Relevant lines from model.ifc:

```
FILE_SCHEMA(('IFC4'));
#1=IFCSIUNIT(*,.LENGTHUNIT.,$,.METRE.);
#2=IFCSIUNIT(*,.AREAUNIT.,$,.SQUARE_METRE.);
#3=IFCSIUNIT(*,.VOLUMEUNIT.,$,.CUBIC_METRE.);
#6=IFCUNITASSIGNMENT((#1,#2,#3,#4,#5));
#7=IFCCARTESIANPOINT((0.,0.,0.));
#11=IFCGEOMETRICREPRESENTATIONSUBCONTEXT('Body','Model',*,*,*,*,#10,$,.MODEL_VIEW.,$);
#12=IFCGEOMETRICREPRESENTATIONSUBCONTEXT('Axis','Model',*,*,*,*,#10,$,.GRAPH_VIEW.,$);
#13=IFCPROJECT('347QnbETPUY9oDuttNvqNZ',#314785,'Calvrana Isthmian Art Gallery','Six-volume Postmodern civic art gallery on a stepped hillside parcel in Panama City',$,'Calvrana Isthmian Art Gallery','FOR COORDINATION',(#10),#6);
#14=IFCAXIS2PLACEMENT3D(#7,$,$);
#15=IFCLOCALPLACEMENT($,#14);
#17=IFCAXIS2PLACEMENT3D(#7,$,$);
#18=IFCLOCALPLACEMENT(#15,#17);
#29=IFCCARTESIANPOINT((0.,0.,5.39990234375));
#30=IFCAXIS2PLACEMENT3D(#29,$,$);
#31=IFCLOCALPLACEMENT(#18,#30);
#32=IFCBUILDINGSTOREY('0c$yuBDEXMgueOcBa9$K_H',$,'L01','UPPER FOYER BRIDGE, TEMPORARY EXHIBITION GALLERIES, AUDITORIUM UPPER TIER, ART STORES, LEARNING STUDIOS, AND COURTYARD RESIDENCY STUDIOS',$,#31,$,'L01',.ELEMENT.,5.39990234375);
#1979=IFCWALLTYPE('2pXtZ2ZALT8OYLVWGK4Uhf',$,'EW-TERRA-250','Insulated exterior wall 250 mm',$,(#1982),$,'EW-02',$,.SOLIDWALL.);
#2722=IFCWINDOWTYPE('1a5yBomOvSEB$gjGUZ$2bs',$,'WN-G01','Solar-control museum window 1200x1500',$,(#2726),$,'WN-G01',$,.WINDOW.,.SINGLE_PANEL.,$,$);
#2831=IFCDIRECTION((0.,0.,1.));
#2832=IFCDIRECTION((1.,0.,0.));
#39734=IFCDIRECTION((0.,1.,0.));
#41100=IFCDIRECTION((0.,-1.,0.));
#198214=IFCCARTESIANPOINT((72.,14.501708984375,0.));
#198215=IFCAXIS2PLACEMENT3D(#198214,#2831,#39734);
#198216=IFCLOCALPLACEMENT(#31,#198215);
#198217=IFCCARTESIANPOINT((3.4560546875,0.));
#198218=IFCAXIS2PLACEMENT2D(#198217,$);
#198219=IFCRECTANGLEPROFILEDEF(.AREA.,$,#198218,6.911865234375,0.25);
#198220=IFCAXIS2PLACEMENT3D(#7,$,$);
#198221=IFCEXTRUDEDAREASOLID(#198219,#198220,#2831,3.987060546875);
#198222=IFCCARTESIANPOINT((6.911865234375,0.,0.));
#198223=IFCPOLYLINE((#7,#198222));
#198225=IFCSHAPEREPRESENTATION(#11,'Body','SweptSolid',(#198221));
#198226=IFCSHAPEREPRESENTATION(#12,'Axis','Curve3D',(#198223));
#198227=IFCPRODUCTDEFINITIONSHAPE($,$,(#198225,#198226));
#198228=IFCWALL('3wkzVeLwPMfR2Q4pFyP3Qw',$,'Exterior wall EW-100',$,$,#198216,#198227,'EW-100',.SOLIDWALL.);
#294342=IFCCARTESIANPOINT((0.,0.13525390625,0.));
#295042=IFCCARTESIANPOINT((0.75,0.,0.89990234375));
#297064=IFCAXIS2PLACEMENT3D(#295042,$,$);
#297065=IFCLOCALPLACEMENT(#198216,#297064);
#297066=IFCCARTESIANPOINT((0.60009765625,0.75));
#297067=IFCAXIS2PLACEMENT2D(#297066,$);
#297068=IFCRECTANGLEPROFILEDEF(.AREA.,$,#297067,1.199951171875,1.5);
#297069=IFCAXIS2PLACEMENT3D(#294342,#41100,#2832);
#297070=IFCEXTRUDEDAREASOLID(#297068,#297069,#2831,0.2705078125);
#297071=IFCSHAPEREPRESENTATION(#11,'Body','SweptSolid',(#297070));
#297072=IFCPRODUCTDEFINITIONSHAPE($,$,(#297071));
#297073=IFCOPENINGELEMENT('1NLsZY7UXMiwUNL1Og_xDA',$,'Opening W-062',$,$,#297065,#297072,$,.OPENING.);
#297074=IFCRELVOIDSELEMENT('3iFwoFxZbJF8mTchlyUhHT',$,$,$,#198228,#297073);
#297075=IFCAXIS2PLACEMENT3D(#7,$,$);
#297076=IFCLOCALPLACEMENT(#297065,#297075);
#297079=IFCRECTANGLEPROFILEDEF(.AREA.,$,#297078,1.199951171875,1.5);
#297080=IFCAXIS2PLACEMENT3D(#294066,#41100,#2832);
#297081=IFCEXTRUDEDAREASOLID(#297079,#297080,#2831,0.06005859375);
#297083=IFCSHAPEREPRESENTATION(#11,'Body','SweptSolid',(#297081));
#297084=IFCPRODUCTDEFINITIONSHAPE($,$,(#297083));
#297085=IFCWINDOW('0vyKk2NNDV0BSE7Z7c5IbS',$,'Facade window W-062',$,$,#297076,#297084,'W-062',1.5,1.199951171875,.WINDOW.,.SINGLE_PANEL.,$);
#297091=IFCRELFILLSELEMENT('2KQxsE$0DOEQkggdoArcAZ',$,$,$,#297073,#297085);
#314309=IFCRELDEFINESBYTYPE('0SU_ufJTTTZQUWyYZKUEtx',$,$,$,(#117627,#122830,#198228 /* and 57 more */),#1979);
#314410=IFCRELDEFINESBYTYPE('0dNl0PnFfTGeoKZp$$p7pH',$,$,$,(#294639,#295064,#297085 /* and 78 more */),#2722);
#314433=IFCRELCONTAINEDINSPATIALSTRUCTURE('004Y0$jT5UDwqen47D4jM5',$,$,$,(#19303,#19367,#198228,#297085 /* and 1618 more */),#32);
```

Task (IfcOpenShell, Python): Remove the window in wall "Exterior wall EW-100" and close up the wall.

```python
import ifcopenshell
import ifcopenshell.api.feature
import ifcopenshell.api.root
import ifcopenshell.geom
import ifcopenshell.util.shape

model = ifcopenshell.open("model.ifc")
settings = ifcopenshell.geom.settings()


def volume(element):
    """Net volume in cubic metres, openings subtracted."""
    shape = ifcopenshell.geom.create_shape(settings, element)
    return ifcopenshell.util.shape.get_volume(shape.geometry)


window = model.by_guid("0vyKk2NNDV0BSE7Z7c5IbS")
opening = window.FillsVoids[0].RelatingOpeningElement
wall = opening.VoidsElements[0].RelatingBuildingElement
before = volume(wall)

ifcopenshell.api.root.remove_product(model, product=window)
ifcopenshell.api.feature.remove_feature(model, feature=opening)

after = volume(wall)

print(f"wall volume {before:.3f} -> {after:.3f} m3")

model.write("model_edited.ifc")
```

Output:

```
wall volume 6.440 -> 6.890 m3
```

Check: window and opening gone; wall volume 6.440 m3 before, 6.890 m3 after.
